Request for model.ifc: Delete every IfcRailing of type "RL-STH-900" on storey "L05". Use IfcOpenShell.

First a look at what the model holds.

```python
import ifcopenshell
import ifcopenshell.util.element

model = ifcopenshell.open("model.ifc")
print(model.schema)
storey = next(s for s in model.by_type("IfcBuildingStorey") if s.Name == "L05")
railings = [e for e in ifcopenshell.util.element.get_decomposition(storey) if e.is_a("IfcRailing")]
seen = {}
for e in railings:
    element_type = ifcopenshell.util.element.get_type(e)
    name = element_type.Name if element_type not in (None, e) else None
    seen[name] = seen.get(name, 0) + 1
for name, count in sorted(seen.items(), key=str):
    print(count, "x", name)
```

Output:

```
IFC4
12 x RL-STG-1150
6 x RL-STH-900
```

```python
import ifcopenshell
import ifcopenshell.api.root
import ifcopenshell.util.element

model = ifcopenshell.open("model.ifc")

storey = next(s for s in model.by_type("IfcBuildingStorey") if s.Name == "L05")
railings = [e for e in ifcopenshell.util.element.get_decomposition(storey) if e.is_a("IfcRailing")]
targets = [e for e in railings if (t := ifcopenshell.util.element.get_type(e)) not in (None, e) and t.Name == "RL-STH-900"]

for e in targets:
    ifcopenshell.api.root.remove_product(model, product=e)
print(len(targets), "removed")

model.write("model_rev.ifc")
```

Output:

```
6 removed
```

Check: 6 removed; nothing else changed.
